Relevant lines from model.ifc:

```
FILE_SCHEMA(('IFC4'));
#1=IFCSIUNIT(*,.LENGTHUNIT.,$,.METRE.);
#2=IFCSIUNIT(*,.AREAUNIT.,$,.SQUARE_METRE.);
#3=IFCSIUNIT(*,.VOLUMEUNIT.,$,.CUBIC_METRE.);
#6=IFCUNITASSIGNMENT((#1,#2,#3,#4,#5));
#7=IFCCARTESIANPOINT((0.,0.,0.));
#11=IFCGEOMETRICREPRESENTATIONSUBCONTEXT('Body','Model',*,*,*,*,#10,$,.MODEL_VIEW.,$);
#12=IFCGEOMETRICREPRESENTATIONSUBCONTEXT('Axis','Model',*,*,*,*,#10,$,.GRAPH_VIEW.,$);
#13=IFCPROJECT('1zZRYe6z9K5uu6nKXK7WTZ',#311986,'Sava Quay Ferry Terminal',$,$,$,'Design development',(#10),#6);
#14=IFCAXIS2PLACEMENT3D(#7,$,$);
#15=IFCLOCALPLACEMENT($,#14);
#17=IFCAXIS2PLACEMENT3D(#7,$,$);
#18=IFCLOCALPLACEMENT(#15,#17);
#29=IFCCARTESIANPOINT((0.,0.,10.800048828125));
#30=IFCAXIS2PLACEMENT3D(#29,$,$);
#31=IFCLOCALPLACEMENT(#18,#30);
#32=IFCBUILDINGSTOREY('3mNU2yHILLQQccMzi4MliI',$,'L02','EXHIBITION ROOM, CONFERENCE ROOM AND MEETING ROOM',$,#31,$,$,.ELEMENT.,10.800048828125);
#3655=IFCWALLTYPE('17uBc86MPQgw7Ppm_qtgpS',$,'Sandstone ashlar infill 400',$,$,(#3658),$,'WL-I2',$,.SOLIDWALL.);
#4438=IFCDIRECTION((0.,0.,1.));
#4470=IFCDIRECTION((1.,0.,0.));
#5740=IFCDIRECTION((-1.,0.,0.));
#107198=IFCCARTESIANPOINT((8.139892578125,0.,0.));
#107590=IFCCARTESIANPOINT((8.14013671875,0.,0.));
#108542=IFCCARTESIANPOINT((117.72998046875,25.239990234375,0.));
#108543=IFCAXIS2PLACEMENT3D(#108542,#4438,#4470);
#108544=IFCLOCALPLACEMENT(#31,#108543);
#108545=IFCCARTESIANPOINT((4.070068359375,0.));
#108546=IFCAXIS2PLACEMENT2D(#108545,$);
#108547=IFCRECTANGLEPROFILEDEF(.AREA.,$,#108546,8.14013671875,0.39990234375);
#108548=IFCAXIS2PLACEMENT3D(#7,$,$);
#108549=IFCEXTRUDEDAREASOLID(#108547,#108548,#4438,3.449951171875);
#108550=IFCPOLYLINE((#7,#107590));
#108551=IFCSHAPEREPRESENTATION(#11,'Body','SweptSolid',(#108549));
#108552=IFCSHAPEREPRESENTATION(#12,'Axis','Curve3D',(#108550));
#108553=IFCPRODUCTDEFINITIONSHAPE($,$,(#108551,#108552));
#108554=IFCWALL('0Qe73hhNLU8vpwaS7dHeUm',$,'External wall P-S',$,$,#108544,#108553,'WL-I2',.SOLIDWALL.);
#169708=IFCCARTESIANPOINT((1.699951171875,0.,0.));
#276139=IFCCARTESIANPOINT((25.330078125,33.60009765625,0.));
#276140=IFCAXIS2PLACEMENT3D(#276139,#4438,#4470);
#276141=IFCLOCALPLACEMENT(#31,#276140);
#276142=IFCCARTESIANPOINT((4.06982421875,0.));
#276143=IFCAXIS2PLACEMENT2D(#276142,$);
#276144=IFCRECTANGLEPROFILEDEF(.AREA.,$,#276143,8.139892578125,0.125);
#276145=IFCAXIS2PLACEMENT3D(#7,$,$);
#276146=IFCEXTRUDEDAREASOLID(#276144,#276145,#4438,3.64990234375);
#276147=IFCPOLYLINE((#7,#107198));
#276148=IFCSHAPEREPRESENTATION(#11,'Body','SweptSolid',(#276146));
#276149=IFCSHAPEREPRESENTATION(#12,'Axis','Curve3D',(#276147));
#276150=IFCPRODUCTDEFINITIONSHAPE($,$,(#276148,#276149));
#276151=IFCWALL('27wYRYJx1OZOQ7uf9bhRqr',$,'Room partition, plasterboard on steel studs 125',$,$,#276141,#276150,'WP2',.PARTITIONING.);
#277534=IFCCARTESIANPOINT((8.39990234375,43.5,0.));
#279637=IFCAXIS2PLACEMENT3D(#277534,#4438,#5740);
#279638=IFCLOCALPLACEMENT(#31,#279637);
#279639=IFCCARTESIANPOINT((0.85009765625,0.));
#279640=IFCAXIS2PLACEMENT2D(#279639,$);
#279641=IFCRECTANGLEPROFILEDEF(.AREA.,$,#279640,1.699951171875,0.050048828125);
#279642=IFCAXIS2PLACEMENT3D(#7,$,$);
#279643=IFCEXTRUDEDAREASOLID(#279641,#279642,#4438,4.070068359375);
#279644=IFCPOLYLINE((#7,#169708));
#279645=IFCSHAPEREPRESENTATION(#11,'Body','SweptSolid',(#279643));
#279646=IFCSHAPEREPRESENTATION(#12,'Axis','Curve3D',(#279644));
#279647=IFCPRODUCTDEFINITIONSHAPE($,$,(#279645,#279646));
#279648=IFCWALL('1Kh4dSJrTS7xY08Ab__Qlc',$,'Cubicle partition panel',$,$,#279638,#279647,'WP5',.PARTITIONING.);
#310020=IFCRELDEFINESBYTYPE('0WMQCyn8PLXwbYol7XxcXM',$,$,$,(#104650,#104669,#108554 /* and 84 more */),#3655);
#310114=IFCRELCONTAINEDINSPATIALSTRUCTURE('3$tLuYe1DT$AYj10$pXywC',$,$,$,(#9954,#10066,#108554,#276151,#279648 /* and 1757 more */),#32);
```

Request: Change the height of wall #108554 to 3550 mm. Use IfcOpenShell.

```python
import ifcopenshell
import ifcopenshell.geom
import ifcopenshell.util.representation
import ifcopenshell.util.shape
import ifcopenshell.util.unit

model = ifcopenshell.open("model.ifc")
unit_scale = ifcopenshell.util.unit.calculate_unit_scale(model)
settings = ifcopenshell.geom.settings()


def volume(element):
    """Net volume in cubic metres, openings subtracted."""
    shape = ifcopenshell.geom.create_shape(settings, element)
    return ifcopenshell.util.shape.get_volume(shape.geometry)


wall = model.by_guid("0Qe73hhNLU8vpwaS7dHeUm")
before = volume(wall)

body = ifcopenshell.util.representation.get_representation(wall, "Model", "Body")
solid = body.Items[0]
old_height = solid.Depth
solid.Depth = 3.55 / unit_scale
after = volume(wall)

print(f"height {old_height:g} -> {solid.Depth:g}, volume {before:.3f} -> {after:.3f} m3")

model.write("model_edited.ifc")
```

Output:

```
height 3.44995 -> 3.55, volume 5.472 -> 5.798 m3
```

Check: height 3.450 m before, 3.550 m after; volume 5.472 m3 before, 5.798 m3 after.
